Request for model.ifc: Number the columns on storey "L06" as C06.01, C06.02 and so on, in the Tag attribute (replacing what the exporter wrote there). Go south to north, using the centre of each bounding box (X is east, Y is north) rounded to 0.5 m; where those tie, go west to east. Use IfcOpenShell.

First a look at what the model holds.

```python
import ifcopenshell
import ifcopenshell.util.element
import ifcopenshell.util.placement

model = ifcopenshell.open("model.ifc")
print(model.schema)
storey = next(s for s in model.by_type("IfcBuildingStorey") if s.Name == "L06")
columns = [e for e in ifcopenshell.util.element.get_decomposition(storey) if e.is_a("IfcColumn")]
for e in sorted(columns, key=lambda e: e.id()):
    origin = ifcopenshell.util.placement.get_local_placement(e.ObjectPlacement)[:3, 3]
    print(e.id(), e.Tag, e.Name, origin.round(2) + 0.0, sep=" | ")
```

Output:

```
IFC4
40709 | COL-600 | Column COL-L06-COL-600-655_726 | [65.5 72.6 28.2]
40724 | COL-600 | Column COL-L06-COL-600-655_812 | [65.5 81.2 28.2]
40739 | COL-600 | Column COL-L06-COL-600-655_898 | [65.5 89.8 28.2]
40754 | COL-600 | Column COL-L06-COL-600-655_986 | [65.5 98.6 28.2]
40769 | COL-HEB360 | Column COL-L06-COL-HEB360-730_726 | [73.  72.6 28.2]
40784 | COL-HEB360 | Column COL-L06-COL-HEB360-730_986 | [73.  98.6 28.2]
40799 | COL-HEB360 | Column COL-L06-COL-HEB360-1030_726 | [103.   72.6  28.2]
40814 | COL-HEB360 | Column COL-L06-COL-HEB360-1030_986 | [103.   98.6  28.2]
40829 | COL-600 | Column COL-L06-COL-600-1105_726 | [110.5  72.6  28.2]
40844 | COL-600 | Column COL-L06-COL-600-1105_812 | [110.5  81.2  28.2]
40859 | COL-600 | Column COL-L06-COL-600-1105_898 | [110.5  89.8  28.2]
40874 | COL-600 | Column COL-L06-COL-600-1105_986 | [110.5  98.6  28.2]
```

```python
import ifcopenshell
import ifcopenshell.geom
import ifcopenshell.util.element
import ifcopenshell.util.shape

model = ifcopenshell.open("model.ifc")
settings = ifcopenshell.geom.settings()
settings.set("use-world-coords", True)


def centre(element):
    shape = ifcopenshell.geom.create_shape(settings, element)
    return ifcopenshell.util.shape.get_bbox_centroid(shape.geometry)


storey = next(s for s in model.by_type("IfcBuildingStorey") if s.Name == "L06")
columns = [e for e in ifcopenshell.util.element.get_decomposition(storey) if e.is_a("IfcColumn")]

# Insertion points can sit at a corner or the storey origin, so sort by the geometry (in metres).
centres = {e: centre(e) for e in columns}
columns.sort(key=lambda e: (round(centres[e][1] / 0.5), centres[e][0]))

for i, e in enumerate(columns, start=1):
    number = f"C06.{i:02d}"
    e.Tag = number
    print(e.id(), number)

model.write("model_v2.ifc")
```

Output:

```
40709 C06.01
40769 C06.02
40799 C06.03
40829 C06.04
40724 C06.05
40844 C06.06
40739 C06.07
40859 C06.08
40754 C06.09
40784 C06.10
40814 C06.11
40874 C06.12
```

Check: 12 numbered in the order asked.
